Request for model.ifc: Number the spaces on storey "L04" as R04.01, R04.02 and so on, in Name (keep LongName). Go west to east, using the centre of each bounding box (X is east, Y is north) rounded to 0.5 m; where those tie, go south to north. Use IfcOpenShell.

First a look at what the model holds.

```python
import ifcopenshell
import ifcopenshell.util.element
import ifcopenshell.util.placement

model = ifcopenshell.open("model.ifc")
print(model.schema)
storey = next(s for s in model.by_type("IfcBuildingStorey") if s.Name == "L04")
spaces = [e for e in ifcopenshell.util.element.get_decomposition(storey) if e.is_a("IfcSpace")]
for e in sorted(spaces, key=lambda e: e.id()):
    origin = ifcopenshell.util.placement.get_local_placement(e.ObjectPlacement)[:3, 3]
    print(e.id(), e.Name, e.LongName, origin.round(2) + 0.0, sep=" | ")
```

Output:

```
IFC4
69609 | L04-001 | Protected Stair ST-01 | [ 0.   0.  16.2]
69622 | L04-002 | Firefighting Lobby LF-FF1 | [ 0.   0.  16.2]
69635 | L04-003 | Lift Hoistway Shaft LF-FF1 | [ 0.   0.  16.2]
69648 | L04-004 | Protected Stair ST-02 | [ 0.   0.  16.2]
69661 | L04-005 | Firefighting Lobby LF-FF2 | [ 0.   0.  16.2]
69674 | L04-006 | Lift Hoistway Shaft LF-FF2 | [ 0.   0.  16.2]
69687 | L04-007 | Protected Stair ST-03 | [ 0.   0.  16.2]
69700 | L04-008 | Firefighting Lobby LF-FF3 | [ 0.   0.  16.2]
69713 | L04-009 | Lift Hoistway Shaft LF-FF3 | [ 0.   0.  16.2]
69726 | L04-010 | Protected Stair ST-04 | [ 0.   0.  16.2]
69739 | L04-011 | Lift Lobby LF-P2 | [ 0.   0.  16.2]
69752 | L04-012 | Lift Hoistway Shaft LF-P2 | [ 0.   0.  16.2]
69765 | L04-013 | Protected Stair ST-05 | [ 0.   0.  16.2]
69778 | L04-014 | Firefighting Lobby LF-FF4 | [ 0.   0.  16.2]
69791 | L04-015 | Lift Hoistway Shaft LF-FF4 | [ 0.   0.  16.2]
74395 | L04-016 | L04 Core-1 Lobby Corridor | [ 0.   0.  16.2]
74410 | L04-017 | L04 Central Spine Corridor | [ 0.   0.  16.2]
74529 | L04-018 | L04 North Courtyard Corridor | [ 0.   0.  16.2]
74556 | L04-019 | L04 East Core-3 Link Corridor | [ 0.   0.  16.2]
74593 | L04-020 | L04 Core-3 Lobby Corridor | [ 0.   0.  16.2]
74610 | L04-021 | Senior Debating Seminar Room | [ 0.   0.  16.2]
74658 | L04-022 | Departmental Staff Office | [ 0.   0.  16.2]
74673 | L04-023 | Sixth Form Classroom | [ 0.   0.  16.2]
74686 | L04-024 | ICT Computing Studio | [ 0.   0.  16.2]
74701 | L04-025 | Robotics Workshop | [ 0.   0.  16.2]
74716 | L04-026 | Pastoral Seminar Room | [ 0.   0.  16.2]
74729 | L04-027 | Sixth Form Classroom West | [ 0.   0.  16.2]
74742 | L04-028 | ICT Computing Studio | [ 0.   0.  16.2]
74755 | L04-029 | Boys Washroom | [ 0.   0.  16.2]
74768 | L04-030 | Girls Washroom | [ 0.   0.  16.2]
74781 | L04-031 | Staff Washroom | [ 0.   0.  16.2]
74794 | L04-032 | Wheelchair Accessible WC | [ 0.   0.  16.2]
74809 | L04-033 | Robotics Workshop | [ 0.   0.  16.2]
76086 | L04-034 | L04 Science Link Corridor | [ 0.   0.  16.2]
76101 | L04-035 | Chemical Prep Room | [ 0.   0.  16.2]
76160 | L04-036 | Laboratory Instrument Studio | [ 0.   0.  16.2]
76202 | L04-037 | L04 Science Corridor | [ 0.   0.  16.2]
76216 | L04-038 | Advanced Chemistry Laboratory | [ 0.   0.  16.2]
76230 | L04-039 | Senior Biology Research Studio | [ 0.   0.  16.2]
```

```python
import ifcopenshell
import ifcopenshell.geom
import ifcopenshell.util.element
import ifcopenshell.util.shape

model = ifcopenshell.open("model.ifc")
settings = ifcopenshell.geom.settings()
settings.set("use-world-coords", True)


def centre(element):
    shape = ifcopenshell.geom.create_shape(settings, element)
    return ifcopenshell.util.shape.get_bbox_centroid(shape.geometry)


storey = next(s for s in model.by_type("IfcBuildingStorey") if s.Name == "L04")
spaces = [e for e in ifcopenshell.util.element.get_decomposition(storey) if e.is_a("IfcSpace")]

# Insertion points can sit at a corner or the storey origin, so sort by the geometry (in metres).
centres = {e: centre(e) for e in spaces}
spaces.sort(key=lambda e: (round(centres[e][0] / 0.5), centres[e][1]))

for i, e in enumerate(spaces, start=1):
    number = f"R04.{i:02d}"
    e.Name = number
    print(e.id(), number)

model.write("model_updated.ifc")
```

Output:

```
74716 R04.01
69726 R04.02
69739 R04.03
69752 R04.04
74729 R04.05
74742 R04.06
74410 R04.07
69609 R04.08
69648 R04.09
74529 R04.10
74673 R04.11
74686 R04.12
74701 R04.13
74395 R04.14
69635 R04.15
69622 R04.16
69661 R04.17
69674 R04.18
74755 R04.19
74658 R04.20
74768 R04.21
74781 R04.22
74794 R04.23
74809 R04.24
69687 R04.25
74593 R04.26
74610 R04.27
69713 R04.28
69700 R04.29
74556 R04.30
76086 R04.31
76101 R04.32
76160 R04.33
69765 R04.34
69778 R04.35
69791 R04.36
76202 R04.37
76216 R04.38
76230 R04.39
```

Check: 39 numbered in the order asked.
